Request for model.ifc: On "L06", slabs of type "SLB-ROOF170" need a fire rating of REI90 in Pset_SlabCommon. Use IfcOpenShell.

First a look at what the model holds.

```python
import ifcopenshell
import ifcopenshell.util.element

model = ifcopenshell.open("model.ifc")
print(model.schema)
storey = next(s for s in model.by_type("IfcBuildingStorey") if s.Name == "L06")
slabs = [e for e in ifcopenshell.util.element.get_decomposition(storey) if e.is_a("IfcSlab")]
seen = {}
for e in slabs:
    element_type = ifcopenshell.util.element.get_type(e)
    key = (element_type.Name if element_type != e and element_type else None, ifcopenshell.util.element.get_pset(e, "Pset_SlabCommon", "FireRating"))
    seen[key] = seen.get(key, 0) + 1
for (name, value), count in sorted(seen.items(), key=str):
    print(count, "x", name, "|", value)
```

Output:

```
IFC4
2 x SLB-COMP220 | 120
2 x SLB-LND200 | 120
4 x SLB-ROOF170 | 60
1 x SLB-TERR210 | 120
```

```python
import ifcopenshell
import ifcopenshell.api.pset
import ifcopenshell.util.element

model = ifcopenshell.open("model.ifc")

storey = next(s for s in model.by_type("IfcBuildingStorey") if s.Name == "L06")
slabs = [e for e in ifcopenshell.util.element.get_decomposition(storey) if e.is_a("IfcSlab")]

count = 0
for e in slabs:
    element_type = ifcopenshell.util.element.get_type(e)
    if element_type in (None, e) or element_type.Name != "SLB-ROOF170":
        continue
    # add_pset returns the element's existing set when there is one.
    pset = ifcopenshell.api.pset.add_pset(model, product=e, name="Pset_SlabCommon")
    ifcopenshell.api.pset.edit_pset(model, pset=pset, properties={"FireRating": "REI90"})
    count += 1

print(count, "slabs updated")

model.write("model_updated.ifc")
```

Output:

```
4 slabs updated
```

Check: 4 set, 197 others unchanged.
